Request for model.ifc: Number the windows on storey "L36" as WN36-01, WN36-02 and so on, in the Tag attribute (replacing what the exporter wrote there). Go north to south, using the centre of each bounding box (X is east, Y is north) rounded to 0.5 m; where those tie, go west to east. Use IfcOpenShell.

First a look at what the model holds.

```python
import ifcopenshell
import ifcopenshell.util.element
import ifcopenshell.util.placement

model = ifcopenshell.open("model.ifc")
print(model.schema)
storey = next(s for s in model.by_type("IfcBuildingStorey") if s.Name == "L36")
windows = [e for e in ifcopenshell.util.element.get_decomposition(storey) if e.is_a("IfcWindow")]
for e in sorted(windows, key=lambda e: e.id()):
    origin = ifcopenshell.util.placement.get_local_placement(e.ObjectPlacement)[:3, 3]
    print(e.id(), e.Tag, e.Name, origin.round(2) + 0.0, sep=" | ")
```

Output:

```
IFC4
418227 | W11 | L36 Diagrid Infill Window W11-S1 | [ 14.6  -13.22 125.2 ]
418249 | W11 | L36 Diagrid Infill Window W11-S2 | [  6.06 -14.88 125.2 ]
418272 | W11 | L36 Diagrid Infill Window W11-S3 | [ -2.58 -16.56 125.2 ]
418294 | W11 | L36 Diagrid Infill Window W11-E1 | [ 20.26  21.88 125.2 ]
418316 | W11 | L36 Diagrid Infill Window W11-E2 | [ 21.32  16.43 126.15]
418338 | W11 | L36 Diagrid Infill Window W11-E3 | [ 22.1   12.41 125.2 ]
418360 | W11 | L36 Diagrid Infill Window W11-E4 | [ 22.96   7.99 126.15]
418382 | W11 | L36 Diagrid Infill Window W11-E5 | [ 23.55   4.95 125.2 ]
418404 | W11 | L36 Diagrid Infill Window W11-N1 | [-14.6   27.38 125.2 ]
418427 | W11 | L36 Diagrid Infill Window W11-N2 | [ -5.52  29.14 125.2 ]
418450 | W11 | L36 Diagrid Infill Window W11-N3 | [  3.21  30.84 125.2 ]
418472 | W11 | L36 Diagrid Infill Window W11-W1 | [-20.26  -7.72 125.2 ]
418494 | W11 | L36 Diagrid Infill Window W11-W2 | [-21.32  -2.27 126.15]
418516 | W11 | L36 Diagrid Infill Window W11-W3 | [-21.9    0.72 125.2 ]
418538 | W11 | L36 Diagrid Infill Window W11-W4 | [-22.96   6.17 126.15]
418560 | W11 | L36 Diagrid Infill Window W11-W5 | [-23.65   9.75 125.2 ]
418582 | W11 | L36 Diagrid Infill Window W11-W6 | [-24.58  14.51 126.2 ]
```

```python
import ifcopenshell
import ifcopenshell.geom
import ifcopenshell.util.element
import ifcopenshell.util.shape

model = ifcopenshell.open("model.ifc")
settings = ifcopenshell.geom.settings()
settings.set("use-world-coords", True)


def centre(element):
    shape = ifcopenshell.geom.create_shape(settings, element)
    return ifcopenshell.util.shape.get_bbox_centroid(shape.geometry)


storey = next(s for s in model.by_type("IfcBuildingStorey") if s.Name == "L36")
windows = [e for e in ifcopenshell.util.element.get_decomposition(storey) if e.is_a("IfcWindow")]

# Insertion points can sit at a corner or the storey origin, so sort by the geometry (in metres).
centres = {e: centre(e) for e in windows}
windows.sort(key=lambda e: (-round(centres[e][1] / 0.5), centres[e][0]))

for i, e in enumerate(windows, start=1):
    number = f"WN36-{i:02d}"
    e.Tag = number
    print(e.id(), number)

model.write("model_v2.ifc")
```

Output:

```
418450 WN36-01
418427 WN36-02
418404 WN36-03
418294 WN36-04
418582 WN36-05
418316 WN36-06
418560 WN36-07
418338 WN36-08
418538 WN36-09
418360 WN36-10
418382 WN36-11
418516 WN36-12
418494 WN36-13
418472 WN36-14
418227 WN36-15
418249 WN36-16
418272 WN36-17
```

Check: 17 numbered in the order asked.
